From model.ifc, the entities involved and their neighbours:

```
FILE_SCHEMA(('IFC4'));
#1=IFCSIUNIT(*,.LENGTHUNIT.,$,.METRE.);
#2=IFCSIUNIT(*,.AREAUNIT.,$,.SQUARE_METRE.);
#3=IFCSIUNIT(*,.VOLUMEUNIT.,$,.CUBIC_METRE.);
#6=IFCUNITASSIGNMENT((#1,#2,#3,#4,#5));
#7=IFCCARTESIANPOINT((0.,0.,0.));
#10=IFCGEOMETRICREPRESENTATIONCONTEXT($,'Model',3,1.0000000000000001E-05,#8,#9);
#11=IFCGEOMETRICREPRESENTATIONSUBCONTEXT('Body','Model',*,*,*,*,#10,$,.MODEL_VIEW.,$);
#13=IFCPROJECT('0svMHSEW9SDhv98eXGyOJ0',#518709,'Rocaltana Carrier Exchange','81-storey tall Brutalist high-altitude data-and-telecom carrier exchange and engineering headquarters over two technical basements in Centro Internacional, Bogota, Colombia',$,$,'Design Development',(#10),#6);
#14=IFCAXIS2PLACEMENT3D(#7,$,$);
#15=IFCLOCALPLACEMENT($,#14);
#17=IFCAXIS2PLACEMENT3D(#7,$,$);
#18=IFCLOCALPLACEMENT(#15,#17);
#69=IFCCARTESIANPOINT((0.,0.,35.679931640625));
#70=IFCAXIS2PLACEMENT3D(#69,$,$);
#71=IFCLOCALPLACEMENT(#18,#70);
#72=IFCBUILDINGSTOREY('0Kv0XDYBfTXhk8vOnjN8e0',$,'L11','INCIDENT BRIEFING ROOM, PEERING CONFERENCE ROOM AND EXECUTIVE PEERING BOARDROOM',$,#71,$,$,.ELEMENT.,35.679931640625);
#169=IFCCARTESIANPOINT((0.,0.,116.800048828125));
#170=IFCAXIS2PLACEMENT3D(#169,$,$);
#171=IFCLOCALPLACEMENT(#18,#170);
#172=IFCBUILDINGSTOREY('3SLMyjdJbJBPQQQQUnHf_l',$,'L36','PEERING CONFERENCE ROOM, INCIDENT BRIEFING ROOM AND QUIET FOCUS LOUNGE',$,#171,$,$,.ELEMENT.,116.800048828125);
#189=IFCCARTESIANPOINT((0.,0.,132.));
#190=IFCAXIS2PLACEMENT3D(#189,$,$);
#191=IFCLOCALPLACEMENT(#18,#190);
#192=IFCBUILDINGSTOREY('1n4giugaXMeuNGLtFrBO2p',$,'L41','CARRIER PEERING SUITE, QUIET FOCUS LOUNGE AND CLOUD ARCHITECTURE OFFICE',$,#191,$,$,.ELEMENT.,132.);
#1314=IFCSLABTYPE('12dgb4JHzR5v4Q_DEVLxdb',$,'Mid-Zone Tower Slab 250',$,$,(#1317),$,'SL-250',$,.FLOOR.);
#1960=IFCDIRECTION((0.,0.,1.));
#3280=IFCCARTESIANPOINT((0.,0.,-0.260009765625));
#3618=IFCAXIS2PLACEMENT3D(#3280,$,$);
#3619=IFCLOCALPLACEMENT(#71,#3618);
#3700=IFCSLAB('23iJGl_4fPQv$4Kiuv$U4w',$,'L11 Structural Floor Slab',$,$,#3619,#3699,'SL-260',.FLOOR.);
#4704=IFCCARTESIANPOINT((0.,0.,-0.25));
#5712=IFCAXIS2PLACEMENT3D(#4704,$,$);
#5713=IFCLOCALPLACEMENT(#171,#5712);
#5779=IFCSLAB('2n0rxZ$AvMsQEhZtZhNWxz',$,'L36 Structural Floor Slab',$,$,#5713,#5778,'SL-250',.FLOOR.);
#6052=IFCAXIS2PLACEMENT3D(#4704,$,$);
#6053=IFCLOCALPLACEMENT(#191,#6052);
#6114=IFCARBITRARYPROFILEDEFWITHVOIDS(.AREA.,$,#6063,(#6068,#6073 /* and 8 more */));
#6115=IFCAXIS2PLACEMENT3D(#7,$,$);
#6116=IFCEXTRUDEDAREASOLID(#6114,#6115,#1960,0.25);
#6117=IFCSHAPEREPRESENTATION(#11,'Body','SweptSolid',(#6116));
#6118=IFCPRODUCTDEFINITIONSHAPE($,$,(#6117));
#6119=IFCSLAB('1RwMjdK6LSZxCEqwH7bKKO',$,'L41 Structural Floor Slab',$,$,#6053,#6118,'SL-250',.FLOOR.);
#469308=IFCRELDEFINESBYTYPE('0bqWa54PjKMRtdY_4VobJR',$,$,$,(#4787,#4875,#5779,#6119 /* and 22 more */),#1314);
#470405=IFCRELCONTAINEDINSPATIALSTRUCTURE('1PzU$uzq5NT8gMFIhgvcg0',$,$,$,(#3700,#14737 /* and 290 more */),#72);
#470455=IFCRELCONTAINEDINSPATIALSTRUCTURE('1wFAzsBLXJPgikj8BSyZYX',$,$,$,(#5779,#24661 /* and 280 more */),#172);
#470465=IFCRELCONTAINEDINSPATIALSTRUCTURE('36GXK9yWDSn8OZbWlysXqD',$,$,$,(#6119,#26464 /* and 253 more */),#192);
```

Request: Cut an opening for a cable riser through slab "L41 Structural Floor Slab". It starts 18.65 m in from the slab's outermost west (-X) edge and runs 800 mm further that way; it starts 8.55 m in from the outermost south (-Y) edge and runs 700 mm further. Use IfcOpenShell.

```python
import numpy as np
import ifcopenshell
import ifcopenshell.api.feature
import ifcopenshell.api.geometry
import ifcopenshell.api.root
import ifcopenshell.geom
import ifcopenshell.util.placement
import ifcopenshell.util.representation
import ifcopenshell.util.shape
import ifcopenshell.util.unit

model = ifcopenshell.open("model.ifc")
unit_scale = ifcopenshell.util.unit.calculate_unit_scale(model)
settings = ifcopenshell.geom.settings()


def volume(element):
    """Net volume in cubic metres, openings subtracted."""
    shape = ifcopenshell.geom.create_shape(settings, element)
    return ifcopenshell.util.shape.get_volume(shape.geometry)


slab = model.by_guid("1RwMjdK6LSZxCEqwH7bKKO")
before = volume(slab)

# Extent in the slab's own axes, in metres. The edges named are its -X and -Y sides.
slab_shape = ifcopenshell.geom.create_shape(settings, slab)
vertices = ifcopenshell.util.shape.get_vertices(slab_shape.geometry)
x_min, y_min, bottom = vertices.min(axis=0)
top = vertices[:, 2].max()

opening = ifcopenshell.api.root.create_entity(model, ifc_class="IfcOpeningElement", name="Cable riser opening", predefined_type="OPENING")
context = ifcopenshell.util.representation.get_context(model, "Model", "Body", "MODEL_VIEW")
width, depth = 0.8, 0.7
outline = [(0.0, 0.0), (width, 0.0), (width, depth), (0.0, depth), (0.0, 0.0)]
# Overshoot both faces by 50 mm so the cut is clean.
shape = ifcopenshell.api.geometry.add_slab_representation(
    model, context=context, depth=top - bottom + 0.1, polyline=outline
)
ifcopenshell.api.geometry.assign_representation(model, product=opening, representation=shape)

matrix = ifcopenshell.util.placement.get_local_placement(slab.ObjectPlacement)
matrix[:, 3] = matrix @ np.append(np.array([x_min + 18.65, y_min + 8.55, bottom - 0.05]) / unit_scale, 1.0)
ifcopenshell.api.geometry.edit_object_placement(model, product=opening, matrix=matrix, is_si=False)
ifcopenshell.api.feature.add_feature(model, feature=opening, element=slab)

after = volume(slab)

print(f"slab volume {before:.3f} -> {after:.3f} m3")

model.write("model_edited.ifc")
```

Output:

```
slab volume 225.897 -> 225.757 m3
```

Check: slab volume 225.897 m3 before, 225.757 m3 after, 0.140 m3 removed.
